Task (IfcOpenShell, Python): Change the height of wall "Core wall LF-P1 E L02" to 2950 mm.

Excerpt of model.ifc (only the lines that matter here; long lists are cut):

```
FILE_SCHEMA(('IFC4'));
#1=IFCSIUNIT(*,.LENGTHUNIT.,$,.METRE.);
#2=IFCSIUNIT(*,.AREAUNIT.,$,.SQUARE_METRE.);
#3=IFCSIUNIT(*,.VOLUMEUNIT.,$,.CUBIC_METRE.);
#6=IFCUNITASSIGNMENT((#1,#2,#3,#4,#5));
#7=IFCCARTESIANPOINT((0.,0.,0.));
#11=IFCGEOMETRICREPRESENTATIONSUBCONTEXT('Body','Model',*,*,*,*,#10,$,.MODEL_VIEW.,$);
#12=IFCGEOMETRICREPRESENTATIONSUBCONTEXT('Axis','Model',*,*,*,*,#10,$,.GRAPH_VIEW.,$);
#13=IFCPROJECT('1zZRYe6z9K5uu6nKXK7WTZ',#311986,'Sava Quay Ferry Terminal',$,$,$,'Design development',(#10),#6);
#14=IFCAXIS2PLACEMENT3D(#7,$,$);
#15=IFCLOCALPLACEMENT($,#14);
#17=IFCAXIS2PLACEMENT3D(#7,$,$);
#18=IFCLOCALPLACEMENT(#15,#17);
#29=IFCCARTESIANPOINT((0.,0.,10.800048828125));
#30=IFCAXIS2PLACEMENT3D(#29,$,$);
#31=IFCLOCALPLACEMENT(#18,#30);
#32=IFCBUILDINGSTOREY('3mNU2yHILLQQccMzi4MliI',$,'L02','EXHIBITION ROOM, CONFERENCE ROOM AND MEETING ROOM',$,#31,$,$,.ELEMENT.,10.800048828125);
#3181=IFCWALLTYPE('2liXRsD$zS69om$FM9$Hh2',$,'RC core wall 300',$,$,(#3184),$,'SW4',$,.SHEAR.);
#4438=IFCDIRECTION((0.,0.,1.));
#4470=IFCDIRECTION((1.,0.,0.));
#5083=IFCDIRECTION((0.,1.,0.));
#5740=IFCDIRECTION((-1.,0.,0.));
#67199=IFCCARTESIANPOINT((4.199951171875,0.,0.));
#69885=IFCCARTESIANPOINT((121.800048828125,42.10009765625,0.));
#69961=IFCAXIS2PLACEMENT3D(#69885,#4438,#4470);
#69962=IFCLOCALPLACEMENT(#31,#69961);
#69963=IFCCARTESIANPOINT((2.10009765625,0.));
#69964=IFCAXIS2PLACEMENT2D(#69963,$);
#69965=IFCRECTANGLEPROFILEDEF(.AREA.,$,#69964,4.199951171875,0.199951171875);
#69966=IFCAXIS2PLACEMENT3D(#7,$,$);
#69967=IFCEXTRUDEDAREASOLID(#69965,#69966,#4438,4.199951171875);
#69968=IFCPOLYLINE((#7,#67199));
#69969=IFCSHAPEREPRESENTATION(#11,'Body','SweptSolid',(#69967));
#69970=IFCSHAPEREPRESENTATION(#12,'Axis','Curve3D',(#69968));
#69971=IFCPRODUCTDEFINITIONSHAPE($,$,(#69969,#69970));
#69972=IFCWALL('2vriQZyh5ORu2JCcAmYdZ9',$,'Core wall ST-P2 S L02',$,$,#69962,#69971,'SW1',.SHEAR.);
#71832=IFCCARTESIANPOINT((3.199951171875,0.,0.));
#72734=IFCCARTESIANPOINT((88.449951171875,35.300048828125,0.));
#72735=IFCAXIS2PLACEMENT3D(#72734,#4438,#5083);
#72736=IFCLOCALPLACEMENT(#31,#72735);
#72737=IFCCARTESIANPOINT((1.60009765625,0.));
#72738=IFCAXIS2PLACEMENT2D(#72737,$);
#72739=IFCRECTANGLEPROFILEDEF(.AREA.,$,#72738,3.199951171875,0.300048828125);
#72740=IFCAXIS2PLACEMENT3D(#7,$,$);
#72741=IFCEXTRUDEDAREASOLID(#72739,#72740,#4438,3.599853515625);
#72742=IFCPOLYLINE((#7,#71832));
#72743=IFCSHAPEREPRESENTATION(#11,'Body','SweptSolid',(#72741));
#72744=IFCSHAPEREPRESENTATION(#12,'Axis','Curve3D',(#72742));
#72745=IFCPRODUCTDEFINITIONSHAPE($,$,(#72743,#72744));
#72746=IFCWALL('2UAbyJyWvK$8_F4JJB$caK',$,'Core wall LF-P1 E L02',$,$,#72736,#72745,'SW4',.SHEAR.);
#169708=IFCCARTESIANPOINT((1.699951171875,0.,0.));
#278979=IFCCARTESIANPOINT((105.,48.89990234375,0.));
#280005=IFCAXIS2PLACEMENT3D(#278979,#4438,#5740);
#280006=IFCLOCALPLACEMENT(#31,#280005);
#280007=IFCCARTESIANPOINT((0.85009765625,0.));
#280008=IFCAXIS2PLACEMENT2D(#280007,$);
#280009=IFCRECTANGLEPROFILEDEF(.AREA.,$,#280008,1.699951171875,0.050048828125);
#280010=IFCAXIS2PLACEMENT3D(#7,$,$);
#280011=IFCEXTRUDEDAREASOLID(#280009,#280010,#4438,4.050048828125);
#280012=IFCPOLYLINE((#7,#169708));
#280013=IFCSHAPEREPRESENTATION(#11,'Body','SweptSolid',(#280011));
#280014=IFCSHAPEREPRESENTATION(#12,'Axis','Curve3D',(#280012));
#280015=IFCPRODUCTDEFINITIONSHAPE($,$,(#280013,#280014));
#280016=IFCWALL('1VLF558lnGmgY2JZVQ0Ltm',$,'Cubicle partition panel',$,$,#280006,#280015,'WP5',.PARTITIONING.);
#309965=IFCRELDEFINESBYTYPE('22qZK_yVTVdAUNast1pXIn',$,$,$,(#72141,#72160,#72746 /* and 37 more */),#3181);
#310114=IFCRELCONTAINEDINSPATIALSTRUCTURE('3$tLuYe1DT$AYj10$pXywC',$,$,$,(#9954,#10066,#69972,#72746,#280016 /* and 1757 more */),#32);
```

```python
import ifcopenshell
import ifcopenshell.geom
import ifcopenshell.util.representation
import ifcopenshell.util.shape
import ifcopenshell.util.unit

model = ifcopenshell.open("model.ifc")
unit_scale = ifcopenshell.util.unit.calculate_unit_scale(model)
settings = ifcopenshell.geom.settings()


def volume(element):
    """Net volume in cubic metres, openings subtracted."""
    shape = ifcopenshell.geom.create_shape(settings, element)
    return ifcopenshell.util.shape.get_volume(shape.geometry)


wall = model.by_guid("2UAbyJyWvK$8_F4JJB$caK")
before = volume(wall)

body = ifcopenshell.util.representation.get_representation(wall, "Model", "Body")
solid = body.Items[0]
old_height = solid.Depth
solid.Depth = 2.95 / unit_scale
after = volume(wall)

print(f"height {old_height:g} -> {solid.Depth:g}, volume {before:.3f} -> {after:.3f} m3")

model.write("model_v2.ifc")
```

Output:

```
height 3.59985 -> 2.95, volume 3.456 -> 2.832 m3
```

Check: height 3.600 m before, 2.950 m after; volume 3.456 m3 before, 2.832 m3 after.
